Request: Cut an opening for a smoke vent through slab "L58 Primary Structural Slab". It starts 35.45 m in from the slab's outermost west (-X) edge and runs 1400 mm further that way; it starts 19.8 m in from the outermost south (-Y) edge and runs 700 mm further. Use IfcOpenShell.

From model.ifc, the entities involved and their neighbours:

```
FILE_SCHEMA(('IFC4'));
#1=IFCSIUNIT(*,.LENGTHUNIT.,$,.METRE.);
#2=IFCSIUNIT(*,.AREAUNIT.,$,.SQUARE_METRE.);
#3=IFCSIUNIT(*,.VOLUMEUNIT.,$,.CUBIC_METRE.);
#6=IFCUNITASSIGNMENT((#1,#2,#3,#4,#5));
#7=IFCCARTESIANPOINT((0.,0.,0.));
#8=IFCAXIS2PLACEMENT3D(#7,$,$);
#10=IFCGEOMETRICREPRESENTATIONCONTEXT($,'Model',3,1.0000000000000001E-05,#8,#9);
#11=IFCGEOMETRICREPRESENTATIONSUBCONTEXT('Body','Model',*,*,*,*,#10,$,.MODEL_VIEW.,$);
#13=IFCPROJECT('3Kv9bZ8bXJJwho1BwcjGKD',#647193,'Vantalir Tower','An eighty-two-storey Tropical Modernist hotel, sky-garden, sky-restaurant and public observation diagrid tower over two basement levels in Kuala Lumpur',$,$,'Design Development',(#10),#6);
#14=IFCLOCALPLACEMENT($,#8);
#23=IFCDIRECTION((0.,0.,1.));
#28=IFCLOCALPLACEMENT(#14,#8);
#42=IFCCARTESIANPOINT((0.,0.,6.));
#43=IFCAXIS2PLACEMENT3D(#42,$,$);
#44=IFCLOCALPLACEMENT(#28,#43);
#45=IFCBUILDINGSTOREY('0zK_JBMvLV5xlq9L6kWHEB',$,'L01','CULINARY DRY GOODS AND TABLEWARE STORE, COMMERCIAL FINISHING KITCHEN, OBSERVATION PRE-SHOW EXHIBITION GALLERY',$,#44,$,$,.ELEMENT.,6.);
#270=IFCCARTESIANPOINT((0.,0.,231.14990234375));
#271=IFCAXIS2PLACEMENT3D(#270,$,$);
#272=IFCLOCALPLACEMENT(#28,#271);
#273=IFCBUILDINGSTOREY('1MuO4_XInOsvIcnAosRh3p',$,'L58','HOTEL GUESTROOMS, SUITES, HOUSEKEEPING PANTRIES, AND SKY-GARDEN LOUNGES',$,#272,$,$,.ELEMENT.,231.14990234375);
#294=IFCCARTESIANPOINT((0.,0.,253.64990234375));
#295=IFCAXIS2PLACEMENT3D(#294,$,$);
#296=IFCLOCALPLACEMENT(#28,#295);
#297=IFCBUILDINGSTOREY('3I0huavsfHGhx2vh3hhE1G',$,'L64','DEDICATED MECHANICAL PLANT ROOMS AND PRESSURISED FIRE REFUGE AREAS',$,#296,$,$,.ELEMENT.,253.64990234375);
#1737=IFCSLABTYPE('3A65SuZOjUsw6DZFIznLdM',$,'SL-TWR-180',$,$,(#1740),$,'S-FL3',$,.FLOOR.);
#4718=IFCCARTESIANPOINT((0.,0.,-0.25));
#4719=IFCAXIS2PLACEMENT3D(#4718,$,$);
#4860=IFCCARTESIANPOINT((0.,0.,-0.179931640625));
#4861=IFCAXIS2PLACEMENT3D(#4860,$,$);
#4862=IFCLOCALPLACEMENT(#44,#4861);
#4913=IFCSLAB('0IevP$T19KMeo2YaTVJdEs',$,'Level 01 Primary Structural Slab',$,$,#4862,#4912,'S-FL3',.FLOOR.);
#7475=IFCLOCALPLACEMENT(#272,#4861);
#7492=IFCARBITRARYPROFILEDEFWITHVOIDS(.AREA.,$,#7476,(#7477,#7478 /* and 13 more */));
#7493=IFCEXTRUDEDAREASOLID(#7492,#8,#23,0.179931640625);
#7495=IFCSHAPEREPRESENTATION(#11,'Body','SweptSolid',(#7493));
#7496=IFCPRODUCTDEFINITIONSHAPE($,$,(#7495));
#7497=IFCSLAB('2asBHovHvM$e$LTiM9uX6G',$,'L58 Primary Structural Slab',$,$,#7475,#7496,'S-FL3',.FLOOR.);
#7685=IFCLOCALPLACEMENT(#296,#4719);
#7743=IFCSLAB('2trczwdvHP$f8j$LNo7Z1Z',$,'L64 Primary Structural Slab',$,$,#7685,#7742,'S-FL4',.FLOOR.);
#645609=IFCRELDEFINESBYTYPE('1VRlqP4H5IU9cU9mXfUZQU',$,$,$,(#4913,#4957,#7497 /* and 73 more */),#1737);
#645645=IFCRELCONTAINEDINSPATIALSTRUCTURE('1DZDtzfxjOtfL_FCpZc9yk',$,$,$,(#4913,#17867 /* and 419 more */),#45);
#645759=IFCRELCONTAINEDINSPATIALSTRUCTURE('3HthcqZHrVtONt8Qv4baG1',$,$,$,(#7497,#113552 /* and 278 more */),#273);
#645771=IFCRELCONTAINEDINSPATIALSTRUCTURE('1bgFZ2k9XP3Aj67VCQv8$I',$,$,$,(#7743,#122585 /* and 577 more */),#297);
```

```python
import numpy as np
import ifcopenshell
import ifcopenshell.api.feature
import ifcopenshell.api.geometry
import ifcopenshell.api.root
import ifcopenshell.geom
import ifcopenshell.util.placement
import ifcopenshell.util.representation
import ifcopenshell.util.shape
import ifcopenshell.util.unit

model = ifcopenshell.open("model.ifc")
unit_scale = ifcopenshell.util.unit.calculate_unit_scale(model)
settings = ifcopenshell.geom.settings()


def volume(element):
    """Net volume in cubic metres, openings subtracted."""
    shape = ifcopenshell.geom.create_shape(settings, element)
    return ifcopenshell.util.shape.get_volume(shape.geometry)


slab = model.by_guid("2asBHovHvM$e$LTiM9uX6G")
before = volume(slab)

# Extent in the slab's own axes, in metres. The edges named are its -X and -Y sides.
slab_shape = ifcopenshell.geom.create_shape(settings, slab)
vertices = ifcopenshell.util.shape.get_vertices(slab_shape.geometry)
x_min, y_min, bottom = vertices.min(axis=0)
top = vertices[:, 2].max()

opening = ifcopenshell.api.root.create_entity(model, ifc_class="IfcOpeningElement", name="Smoke vent opening", predefined_type="OPENING")
context = ifcopenshell.util.representation.get_context(model, "Model", "Body", "MODEL_VIEW")
width, depth = 1.4, 0.7
outline = [(0.0, 0.0), (width, 0.0), (width, depth), (0.0, depth), (0.0, 0.0)]
# Overshoot both faces by 50 mm so the cut is clean.
shape = ifcopenshell.api.geometry.add_slab_representation(
    model, context=context, depth=top - bottom + 0.1, polyline=outline
)
ifcopenshell.api.geometry.assign_representation(model, product=opening, representation=shape)

matrix = ifcopenshell.util.placement.get_local_placement(slab.ObjectPlacement)
matrix[:, 3] = matrix @ np.append(np.array([x_min + 35.45, y_min + 19.8, bottom - 0.05]) / unit_scale, 1.0)
ifcopenshell.api.geometry.edit_object_placement(model, product=opening, matrix=matrix, is_si=False)
ifcopenshell.api.feature.add_feature(model, feature=opening, element=slab)

after = volume(slab)

print(f"slab volume {before:.3f} -> {after:.3f} m3")

model.write("model_edited.ifc")
```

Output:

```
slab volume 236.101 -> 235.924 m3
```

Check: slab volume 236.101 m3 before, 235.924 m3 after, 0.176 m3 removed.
